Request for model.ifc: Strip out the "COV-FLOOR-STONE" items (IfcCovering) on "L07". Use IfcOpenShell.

First a look at what the model holds.

```python
import ifcopenshell
import ifcopenshell.util.element

model = ifcopenshell.open("model.ifc")
print(model.schema)
storey = next(s for s in model.by_type("IfcBuildingStorey") if s.Name == "L07")
coverings = [e for e in ifcopenshell.util.element.get_decomposition(storey) if e.is_a("IfcCovering")]
seen = {}
for e in coverings:
    element_type = ifcopenshell.util.element.get_type(e)
    name = element_type.Name if element_type not in (None, e) else None
    seen[name] = seen.get(name, 0) + 1
for name, count in sorted(seen.items(), key=str):
    print(count, "x", name)
```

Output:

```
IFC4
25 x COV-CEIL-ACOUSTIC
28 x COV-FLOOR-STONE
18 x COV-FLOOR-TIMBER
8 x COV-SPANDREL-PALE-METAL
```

```python
import ifcopenshell
import ifcopenshell.api.root
import ifcopenshell.util.element

model = ifcopenshell.open("model.ifc")

storey = next(s for s in model.by_type("IfcBuildingStorey") if s.Name == "L07")
coverings = [e for e in ifcopenshell.util.element.get_decomposition(storey) if e.is_a("IfcCovering")]
targets = [e for e in coverings if (t := ifcopenshell.util.element.get_type(e)) not in (None, e) and t.Name == "COV-FLOOR-STONE"]

for e in targets:
    ifcopenshell.api.root.remove_product(model, product=e)
print(len(targets), "removed")

model.write("model_updated.ifc")
```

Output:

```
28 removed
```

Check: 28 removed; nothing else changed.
